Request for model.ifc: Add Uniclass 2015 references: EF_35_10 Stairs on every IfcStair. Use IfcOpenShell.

First a look at what the model holds.

```python
import ifcopenshell

model = ifcopenshell.open("model.ifc")
print(model.schema)
print("classifications:", [c.Name for c in model.by_type("IfcClassification")])
for ifc_class in ("IfcDoor", "IfcRoof", "IfcStair", "IfcWall", "IfcWindow"):
    print(ifc_class, len(model.by_type(ifc_class)))
```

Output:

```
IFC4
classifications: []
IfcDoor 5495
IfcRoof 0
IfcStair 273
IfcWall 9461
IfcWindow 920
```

```python
import ifcopenshell
import ifcopenshell.api.classification

model = ifcopenshell.open("model.ifc")

system = ifcopenshell.api.classification.add_classification(model, classification="Uniclass 2015")

codes = {
    "IfcStair": ("EF_35_10", "Stairs"),
}
for ifc_class, (code, name) in codes.items():
    products = model.by_type(ifc_class)
    ifcopenshell.api.classification.add_reference(
        model, products=products, classification=system, identification=code, name=name
    )
    print(code, len(products))

model.write("model_v2.ifc")
```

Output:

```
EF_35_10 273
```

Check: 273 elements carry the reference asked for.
